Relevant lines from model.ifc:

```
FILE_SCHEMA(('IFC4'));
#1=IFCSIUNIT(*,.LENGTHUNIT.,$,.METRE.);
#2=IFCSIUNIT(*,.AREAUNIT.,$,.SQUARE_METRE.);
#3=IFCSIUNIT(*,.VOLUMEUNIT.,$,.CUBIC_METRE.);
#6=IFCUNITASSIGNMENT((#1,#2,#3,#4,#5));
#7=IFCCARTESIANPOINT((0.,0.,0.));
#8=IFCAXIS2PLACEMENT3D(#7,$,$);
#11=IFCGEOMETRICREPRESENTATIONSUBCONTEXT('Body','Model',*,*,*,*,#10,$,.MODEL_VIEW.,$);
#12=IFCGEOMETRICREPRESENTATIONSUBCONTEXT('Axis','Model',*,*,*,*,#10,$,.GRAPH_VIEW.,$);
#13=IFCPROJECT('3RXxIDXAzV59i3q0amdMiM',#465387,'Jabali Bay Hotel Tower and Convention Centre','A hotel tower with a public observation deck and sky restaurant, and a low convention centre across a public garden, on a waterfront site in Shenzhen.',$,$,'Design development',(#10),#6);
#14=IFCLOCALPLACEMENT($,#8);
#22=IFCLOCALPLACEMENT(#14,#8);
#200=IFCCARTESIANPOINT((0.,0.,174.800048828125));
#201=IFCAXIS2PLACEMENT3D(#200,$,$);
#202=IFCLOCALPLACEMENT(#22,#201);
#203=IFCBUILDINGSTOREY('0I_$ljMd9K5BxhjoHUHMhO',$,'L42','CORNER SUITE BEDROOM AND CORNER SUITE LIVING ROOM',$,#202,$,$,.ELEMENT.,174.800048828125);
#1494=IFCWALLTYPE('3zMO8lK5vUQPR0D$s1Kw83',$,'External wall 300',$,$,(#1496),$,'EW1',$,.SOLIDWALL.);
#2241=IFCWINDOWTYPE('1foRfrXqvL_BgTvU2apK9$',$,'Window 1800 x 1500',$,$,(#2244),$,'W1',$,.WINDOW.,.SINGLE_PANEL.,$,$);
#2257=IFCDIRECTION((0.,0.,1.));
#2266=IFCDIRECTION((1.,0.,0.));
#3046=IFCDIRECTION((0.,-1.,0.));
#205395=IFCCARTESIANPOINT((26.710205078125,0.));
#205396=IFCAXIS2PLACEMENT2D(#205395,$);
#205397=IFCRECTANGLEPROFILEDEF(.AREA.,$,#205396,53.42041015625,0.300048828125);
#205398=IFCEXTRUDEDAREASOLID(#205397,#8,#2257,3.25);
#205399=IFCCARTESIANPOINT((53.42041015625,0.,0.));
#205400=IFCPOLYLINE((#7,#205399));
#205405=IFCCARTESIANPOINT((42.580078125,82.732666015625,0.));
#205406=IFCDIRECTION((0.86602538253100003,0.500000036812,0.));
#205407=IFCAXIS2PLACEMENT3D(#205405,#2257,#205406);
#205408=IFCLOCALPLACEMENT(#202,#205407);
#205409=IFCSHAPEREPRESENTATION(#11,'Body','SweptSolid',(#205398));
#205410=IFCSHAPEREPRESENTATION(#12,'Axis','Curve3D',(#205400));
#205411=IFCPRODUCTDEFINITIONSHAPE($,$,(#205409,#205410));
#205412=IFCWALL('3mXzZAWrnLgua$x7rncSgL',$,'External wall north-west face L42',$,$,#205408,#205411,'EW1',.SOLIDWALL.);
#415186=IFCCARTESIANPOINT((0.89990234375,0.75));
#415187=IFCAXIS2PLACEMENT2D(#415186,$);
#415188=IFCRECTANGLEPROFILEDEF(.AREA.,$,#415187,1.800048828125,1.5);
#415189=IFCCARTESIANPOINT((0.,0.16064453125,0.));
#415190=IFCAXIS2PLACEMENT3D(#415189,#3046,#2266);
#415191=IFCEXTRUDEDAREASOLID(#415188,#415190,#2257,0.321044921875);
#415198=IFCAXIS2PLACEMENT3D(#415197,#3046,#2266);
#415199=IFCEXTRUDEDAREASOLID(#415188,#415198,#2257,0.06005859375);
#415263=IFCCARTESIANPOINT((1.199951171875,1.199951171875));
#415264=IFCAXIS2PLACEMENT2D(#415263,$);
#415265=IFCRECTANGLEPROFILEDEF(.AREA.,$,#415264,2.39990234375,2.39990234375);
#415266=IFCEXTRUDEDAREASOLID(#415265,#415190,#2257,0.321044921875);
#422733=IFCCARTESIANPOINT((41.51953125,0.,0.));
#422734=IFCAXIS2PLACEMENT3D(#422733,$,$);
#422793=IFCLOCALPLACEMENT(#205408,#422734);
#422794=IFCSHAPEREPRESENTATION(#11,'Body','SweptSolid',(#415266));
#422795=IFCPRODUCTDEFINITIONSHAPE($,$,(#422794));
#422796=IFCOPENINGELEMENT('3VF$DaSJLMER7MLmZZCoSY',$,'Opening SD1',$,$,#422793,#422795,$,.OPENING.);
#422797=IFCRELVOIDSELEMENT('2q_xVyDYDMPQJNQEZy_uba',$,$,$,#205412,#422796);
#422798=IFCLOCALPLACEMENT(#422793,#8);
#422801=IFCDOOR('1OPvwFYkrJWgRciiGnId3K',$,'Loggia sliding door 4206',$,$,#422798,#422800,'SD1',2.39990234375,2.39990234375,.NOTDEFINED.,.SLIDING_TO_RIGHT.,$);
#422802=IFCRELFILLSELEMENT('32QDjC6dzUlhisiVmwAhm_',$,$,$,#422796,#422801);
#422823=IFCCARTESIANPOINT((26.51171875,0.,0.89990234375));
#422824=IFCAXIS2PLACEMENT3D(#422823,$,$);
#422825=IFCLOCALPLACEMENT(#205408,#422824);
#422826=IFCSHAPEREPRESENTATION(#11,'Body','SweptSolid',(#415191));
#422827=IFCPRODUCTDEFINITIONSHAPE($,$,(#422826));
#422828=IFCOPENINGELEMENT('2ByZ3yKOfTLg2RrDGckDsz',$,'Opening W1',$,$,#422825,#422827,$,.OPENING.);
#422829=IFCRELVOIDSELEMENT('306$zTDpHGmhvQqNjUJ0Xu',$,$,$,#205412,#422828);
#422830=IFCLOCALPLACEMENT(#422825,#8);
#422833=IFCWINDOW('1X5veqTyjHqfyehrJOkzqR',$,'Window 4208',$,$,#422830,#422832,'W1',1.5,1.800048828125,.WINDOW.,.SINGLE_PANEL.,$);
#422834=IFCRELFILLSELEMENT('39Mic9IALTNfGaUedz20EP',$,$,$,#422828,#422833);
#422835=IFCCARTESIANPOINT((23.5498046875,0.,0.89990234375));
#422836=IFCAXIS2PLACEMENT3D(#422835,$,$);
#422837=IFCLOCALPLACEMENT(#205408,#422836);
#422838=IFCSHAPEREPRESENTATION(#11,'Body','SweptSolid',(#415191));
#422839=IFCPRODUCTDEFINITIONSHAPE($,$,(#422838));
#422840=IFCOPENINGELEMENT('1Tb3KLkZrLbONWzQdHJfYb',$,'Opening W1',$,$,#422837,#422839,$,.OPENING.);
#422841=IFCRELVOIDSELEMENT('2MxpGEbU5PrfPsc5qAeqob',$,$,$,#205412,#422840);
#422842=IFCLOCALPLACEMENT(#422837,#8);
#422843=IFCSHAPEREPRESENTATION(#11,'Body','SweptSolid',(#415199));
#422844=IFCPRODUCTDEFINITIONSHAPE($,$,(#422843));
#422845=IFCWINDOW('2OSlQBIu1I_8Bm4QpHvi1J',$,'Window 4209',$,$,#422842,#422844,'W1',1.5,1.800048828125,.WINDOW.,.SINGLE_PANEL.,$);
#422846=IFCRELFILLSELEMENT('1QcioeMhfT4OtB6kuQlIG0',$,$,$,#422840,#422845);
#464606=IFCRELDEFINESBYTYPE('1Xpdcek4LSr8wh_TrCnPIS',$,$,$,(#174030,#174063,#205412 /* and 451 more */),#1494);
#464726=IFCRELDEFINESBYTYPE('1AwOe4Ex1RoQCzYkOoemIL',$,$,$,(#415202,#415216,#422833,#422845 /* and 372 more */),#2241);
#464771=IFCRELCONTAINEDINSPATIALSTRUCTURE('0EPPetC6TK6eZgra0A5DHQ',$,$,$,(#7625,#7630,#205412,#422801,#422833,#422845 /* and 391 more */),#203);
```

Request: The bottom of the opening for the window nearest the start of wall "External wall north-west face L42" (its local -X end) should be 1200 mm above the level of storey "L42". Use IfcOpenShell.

```python
import numpy as np
import ifcopenshell
import ifcopenshell.api.geometry
import ifcopenshell.geom
import ifcopenshell.util.element
import ifcopenshell.util.placement
import ifcopenshell.util.shape
import ifcopenshell.util.unit

model = ifcopenshell.open("model.ifc")
unit_scale = ifcopenshell.util.unit.calculate_unit_scale(model)

window = model.by_guid("2OSlQBIu1I_8Bm4QpHvi1J")
opening = window.FillsVoids[0].RelatingOpeningElement
storey = ifcopenshell.util.element.get_container(window, ifc_class="IfcBuildingStorey")
level = ifcopenshell.util.placement.get_local_placement(storey.ObjectPlacement)[2, 3]

# The opening's origin need not be at the sill, so measure its lowest point.
shape = ifcopenshell.geom.create_shape(ifcopenshell.geom.settings(), opening)
bottom = ifcopenshell.util.shape.get_shape_bottom_elevation(shape, shape.geometry) / unit_scale
dz = level + 1.2 - bottom

shift = np.array([0.0, 0.0, dz])
# The window is placed relative to its opening, so it follows when the opening moves.
matrix = ifcopenshell.util.placement.get_local_placement(opening.ObjectPlacement)
matrix[:3, 3] += shift
ifcopenshell.api.geometry.edit_object_placement(
    model, product=opening, matrix=matrix, is_si=False, should_transform_children=True
)

print(f"moved by {dz * unit_scale:+.3f} m")

model.write("model_edited.ifc")
```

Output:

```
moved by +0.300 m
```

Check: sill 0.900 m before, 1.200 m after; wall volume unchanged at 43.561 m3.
